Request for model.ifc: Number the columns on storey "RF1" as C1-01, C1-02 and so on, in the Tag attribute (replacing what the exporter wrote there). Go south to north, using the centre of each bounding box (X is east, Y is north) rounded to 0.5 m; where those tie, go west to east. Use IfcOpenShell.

First a look at what the model holds.

```python
import ifcopenshell
import ifcopenshell.util.element
import ifcopenshell.util.placement

model = ifcopenshell.open("model.ifc")
print(model.schema)
storey = next(s for s in model.by_type("IfcBuildingStorey") if s.Name == "RF1")
columns = [e for e in ifcopenshell.util.element.get_decomposition(storey) if e.is_a("IfcColumn")]
for e in sorted(columns, key=lambda e: e.id()):
    origin = ifcopenshell.util.placement.get_local_placement(e.ObjectPlacement)[:3, 3]
    print(e.id(), e.Tag, e.Name, origin.round(2) + 0.0, sep=" | ")
```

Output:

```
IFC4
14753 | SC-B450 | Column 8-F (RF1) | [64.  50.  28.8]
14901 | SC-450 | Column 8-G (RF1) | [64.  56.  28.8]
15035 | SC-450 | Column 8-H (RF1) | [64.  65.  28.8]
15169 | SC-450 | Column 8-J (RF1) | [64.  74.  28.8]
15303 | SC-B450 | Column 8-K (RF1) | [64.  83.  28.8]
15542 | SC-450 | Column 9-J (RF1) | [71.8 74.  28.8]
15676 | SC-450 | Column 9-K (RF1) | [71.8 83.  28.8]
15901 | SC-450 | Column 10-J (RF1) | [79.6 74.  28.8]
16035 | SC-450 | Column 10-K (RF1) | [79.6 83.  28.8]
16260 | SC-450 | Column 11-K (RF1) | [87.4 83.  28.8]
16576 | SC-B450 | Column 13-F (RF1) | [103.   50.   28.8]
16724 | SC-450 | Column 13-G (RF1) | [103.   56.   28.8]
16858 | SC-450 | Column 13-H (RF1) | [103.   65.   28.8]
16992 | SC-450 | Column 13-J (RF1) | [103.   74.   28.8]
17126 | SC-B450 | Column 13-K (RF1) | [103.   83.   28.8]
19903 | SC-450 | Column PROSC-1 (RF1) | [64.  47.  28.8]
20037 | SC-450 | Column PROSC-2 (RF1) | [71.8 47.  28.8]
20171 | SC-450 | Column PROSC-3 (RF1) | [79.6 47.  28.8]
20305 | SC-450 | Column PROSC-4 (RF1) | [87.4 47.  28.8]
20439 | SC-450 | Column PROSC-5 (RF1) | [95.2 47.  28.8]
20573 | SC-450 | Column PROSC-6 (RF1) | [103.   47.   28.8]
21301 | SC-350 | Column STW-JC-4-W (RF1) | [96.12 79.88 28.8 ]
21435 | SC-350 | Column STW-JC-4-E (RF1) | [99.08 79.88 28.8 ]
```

```python
import ifcopenshell
import ifcopenshell.geom
import ifcopenshell.util.element
import ifcopenshell.util.shape

model = ifcopenshell.open("model.ifc")
settings = ifcopenshell.geom.settings()
settings.set("use-world-coords", True)


def centre(element):
    shape = ifcopenshell.geom.create_shape(settings, element)
    return ifcopenshell.util.shape.get_bbox_centroid(shape.geometry)


storey = next(s for s in model.by_type("IfcBuildingStorey") if s.Name == "RF1")
columns = [e for e in ifcopenshell.util.element.get_decomposition(storey) if e.is_a("IfcColumn")]

# Insertion points can sit at a corner or the storey origin, so sort by the geometry (in metres).
centres = {e: centre(e) for e in columns}
columns.sort(key=lambda e: (round(centres[e][1] / 0.5), centres[e][0]))

for i, e in enumerate(columns, start=1):
    number = f"C1-{i:02d}"
    e.Tag = number
    print(e.id(), number)

model.write("model-out.ifc")
```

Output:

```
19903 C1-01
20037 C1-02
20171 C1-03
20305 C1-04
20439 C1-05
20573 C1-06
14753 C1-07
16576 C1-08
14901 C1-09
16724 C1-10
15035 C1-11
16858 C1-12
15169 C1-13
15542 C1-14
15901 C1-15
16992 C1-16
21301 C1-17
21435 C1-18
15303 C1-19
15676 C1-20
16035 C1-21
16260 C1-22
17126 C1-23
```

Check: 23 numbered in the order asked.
